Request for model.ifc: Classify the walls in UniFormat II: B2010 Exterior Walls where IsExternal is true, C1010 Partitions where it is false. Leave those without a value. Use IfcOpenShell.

First a look at what the model holds.

```python
import ifcopenshell
import ifcopenshell.util.element

model = ifcopenshell.open("model.ifc")
print(model.schema)
print("classifications:", [c.Name for c in model.by_type("IfcClassification")])
values = [ifcopenshell.util.element.get_pset(e, "Pset_WallCommon", "IsExternal") for e in model.by_type("IfcWall")]
for value in (True, False, None):
    print("IsExternal", value, values.count(value))
```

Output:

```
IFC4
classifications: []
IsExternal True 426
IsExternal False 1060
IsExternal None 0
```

```python
import ifcopenshell
import ifcopenshell.api.classification
import ifcopenshell.util.element

model = ifcopenshell.open("model.ifc")

system = ifcopenshell.api.classification.add_classification(model, classification="UniFormat II")

walls = model.by_type("IfcWall")
external = {e: ifcopenshell.util.element.get_pset(e, "Pset_WallCommon", "IsExternal") for e in walls}
for flag, code, name in ((True, "B2010", "Exterior Walls"), (False, "C1010", "Partitions")):
    products = [e for e in walls if external[e] is flag]
    ifcopenshell.api.classification.add_reference(
        model, products=products, classification=system, identification=code, name=name
    )
    print(code, len(products))

model.write("model-out.ifc")
```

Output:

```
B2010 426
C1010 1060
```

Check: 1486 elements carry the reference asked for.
